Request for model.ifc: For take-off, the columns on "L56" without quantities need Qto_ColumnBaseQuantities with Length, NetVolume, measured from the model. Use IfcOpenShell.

First a look at what the model holds.

```python
import ifcopenshell
import ifcopenshell.util.element
import ifcopenshell.util.unit

model = ifcopenshell.open("model.ifc")
print(model.schema)
for unit_type in ("LENGTHUNIT", "AREAUNIT", "VOLUMEUNIT"):
    print(unit_type, ifcopenshell.util.unit.calculate_unit_scale(model, unit_type))
storey = next(s for s in model.by_type("IfcBuildingStorey") if s.Name == "L56")
columns = [e for e in ifcopenshell.util.element.get_decomposition(storey) if e.is_a("IfcColumn")]
for e in sorted(columns, key=lambda e: e.id()):
    print(e.id(), e.is_a(), e.Name, list(ifcopenshell.util.element.get_psets(e, qtos_only=True)), sep=" | ")
```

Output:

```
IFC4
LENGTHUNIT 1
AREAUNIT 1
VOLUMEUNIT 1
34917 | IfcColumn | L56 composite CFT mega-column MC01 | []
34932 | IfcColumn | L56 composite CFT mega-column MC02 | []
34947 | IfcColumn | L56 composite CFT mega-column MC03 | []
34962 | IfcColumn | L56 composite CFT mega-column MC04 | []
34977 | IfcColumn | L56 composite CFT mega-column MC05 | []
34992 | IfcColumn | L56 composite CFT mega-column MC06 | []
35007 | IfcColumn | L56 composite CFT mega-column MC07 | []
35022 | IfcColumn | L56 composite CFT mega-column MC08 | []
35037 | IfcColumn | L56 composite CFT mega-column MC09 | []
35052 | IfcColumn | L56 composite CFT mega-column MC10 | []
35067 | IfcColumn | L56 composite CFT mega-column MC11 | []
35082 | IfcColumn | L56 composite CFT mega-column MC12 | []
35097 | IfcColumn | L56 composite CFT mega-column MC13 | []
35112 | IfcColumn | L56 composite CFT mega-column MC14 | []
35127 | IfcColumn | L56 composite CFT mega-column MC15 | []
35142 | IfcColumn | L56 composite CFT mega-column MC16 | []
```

```python
import ifcopenshell
import ifcopenshell.api.pset
import ifcopenshell.geom
import ifcopenshell.util.element
import ifcopenshell.util.shape
import ifcopenshell.util.unit

model = ifcopenshell.open("model.ifc")
unit_scale = ifcopenshell.util.unit.calculate_unit_scale(model)
volume_scale = ifcopenshell.util.unit.calculate_unit_scale(model, "VOLUMEUNIT")
settings = ifcopenshell.geom.settings()

storey = next(s for s in model.by_type("IfcBuildingStorey") if s.Name == "L56")
columns = [e for e in ifcopenshell.util.element.get_decomposition(storey) if e.is_a("IfcColumn")]

for e in sorted(columns, key=lambda e: e.id()):
    if ifcopenshell.util.element.get_psets(e, qtos_only=True, should_inherit=False):
        continue
    # Geometry comes back in metres, in the element's own axes.
    shape = ifcopenshell.geom.create_shape(settings, e)
    values = {
        "Length": ifcopenshell.util.shape.get_z(shape.geometry) / unit_scale,
        "NetVolume": ifcopenshell.util.shape.get_volume(shape.geometry) / volume_scale,
    }
    qto = ifcopenshell.api.pset.add_qto(model, product=e, name="Qto_ColumnBaseQuantities")
    ifcopenshell.api.pset.edit_qto(model, qto=qto, properties=values)
    print(e.id(), {k: round(v, 3) for k, v in values.items()})

model.write("model-out.ifc")
```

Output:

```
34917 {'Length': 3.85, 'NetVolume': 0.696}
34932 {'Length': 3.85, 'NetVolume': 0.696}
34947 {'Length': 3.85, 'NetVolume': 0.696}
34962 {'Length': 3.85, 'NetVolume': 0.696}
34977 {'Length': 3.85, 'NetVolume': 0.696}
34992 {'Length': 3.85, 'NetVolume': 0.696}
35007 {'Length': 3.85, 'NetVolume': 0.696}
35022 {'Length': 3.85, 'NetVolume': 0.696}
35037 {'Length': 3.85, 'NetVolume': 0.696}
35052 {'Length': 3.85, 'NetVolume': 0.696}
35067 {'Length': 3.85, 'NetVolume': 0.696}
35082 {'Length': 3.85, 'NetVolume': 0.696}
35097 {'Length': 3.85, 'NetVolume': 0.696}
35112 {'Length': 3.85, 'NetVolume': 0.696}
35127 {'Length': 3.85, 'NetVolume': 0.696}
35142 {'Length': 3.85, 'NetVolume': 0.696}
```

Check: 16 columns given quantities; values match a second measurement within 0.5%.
